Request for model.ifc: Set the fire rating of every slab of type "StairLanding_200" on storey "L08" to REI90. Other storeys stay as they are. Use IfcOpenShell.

First a look at what the model holds.

```python
import ifcopenshell
import ifcopenshell.util.element

model = ifcopenshell.open("model.ifc")
print(model.schema)
storey = next(s for s in model.by_type("IfcBuildingStorey") if s.Name == "L08")
slabs = [e for e in ifcopenshell.util.element.get_decomposition(storey) if e.is_a("IfcSlab")]
seen = {}
for e in slabs:
    element_type = ifcopenshell.util.element.get_type(e)
    key = (element_type.Name if element_type != e and element_type else None, ifcopenshell.util.element.get_pset(e, "Pset_SlabCommon", "FireRating"))
    seen[key] = seen.get(key, 0) + 1
for (name, value), count in sorted(seen.items(), key=str):
    print(count, "x", name, "|", value)
```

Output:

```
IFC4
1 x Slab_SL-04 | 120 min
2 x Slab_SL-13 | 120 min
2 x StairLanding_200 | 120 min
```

```python
import ifcopenshell
import ifcopenshell.api.pset
import ifcopenshell.util.element

model = ifcopenshell.open("model.ifc")

storey = next(s for s in model.by_type("IfcBuildingStorey") if s.Name == "L08")
slabs = [e for e in ifcopenshell.util.element.get_decomposition(storey) if e.is_a("IfcSlab")]

count = 0
for e in slabs:
    element_type = ifcopenshell.util.element.get_type(e)
    if element_type in (None, e) or element_type.Name != "StairLanding_200":
        continue
    # add_pset returns the element's existing set when there is one.
    pset = ifcopenshell.api.pset.add_pset(model, product=e, name="Pset_SlabCommon")
    ifcopenshell.api.pset.edit_pset(model, pset=pset, properties={"FireRating": "REI90"})
    count += 1

print(count, "slabs updated")

model.write("model_updated.ifc")
```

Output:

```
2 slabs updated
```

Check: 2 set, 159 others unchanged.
